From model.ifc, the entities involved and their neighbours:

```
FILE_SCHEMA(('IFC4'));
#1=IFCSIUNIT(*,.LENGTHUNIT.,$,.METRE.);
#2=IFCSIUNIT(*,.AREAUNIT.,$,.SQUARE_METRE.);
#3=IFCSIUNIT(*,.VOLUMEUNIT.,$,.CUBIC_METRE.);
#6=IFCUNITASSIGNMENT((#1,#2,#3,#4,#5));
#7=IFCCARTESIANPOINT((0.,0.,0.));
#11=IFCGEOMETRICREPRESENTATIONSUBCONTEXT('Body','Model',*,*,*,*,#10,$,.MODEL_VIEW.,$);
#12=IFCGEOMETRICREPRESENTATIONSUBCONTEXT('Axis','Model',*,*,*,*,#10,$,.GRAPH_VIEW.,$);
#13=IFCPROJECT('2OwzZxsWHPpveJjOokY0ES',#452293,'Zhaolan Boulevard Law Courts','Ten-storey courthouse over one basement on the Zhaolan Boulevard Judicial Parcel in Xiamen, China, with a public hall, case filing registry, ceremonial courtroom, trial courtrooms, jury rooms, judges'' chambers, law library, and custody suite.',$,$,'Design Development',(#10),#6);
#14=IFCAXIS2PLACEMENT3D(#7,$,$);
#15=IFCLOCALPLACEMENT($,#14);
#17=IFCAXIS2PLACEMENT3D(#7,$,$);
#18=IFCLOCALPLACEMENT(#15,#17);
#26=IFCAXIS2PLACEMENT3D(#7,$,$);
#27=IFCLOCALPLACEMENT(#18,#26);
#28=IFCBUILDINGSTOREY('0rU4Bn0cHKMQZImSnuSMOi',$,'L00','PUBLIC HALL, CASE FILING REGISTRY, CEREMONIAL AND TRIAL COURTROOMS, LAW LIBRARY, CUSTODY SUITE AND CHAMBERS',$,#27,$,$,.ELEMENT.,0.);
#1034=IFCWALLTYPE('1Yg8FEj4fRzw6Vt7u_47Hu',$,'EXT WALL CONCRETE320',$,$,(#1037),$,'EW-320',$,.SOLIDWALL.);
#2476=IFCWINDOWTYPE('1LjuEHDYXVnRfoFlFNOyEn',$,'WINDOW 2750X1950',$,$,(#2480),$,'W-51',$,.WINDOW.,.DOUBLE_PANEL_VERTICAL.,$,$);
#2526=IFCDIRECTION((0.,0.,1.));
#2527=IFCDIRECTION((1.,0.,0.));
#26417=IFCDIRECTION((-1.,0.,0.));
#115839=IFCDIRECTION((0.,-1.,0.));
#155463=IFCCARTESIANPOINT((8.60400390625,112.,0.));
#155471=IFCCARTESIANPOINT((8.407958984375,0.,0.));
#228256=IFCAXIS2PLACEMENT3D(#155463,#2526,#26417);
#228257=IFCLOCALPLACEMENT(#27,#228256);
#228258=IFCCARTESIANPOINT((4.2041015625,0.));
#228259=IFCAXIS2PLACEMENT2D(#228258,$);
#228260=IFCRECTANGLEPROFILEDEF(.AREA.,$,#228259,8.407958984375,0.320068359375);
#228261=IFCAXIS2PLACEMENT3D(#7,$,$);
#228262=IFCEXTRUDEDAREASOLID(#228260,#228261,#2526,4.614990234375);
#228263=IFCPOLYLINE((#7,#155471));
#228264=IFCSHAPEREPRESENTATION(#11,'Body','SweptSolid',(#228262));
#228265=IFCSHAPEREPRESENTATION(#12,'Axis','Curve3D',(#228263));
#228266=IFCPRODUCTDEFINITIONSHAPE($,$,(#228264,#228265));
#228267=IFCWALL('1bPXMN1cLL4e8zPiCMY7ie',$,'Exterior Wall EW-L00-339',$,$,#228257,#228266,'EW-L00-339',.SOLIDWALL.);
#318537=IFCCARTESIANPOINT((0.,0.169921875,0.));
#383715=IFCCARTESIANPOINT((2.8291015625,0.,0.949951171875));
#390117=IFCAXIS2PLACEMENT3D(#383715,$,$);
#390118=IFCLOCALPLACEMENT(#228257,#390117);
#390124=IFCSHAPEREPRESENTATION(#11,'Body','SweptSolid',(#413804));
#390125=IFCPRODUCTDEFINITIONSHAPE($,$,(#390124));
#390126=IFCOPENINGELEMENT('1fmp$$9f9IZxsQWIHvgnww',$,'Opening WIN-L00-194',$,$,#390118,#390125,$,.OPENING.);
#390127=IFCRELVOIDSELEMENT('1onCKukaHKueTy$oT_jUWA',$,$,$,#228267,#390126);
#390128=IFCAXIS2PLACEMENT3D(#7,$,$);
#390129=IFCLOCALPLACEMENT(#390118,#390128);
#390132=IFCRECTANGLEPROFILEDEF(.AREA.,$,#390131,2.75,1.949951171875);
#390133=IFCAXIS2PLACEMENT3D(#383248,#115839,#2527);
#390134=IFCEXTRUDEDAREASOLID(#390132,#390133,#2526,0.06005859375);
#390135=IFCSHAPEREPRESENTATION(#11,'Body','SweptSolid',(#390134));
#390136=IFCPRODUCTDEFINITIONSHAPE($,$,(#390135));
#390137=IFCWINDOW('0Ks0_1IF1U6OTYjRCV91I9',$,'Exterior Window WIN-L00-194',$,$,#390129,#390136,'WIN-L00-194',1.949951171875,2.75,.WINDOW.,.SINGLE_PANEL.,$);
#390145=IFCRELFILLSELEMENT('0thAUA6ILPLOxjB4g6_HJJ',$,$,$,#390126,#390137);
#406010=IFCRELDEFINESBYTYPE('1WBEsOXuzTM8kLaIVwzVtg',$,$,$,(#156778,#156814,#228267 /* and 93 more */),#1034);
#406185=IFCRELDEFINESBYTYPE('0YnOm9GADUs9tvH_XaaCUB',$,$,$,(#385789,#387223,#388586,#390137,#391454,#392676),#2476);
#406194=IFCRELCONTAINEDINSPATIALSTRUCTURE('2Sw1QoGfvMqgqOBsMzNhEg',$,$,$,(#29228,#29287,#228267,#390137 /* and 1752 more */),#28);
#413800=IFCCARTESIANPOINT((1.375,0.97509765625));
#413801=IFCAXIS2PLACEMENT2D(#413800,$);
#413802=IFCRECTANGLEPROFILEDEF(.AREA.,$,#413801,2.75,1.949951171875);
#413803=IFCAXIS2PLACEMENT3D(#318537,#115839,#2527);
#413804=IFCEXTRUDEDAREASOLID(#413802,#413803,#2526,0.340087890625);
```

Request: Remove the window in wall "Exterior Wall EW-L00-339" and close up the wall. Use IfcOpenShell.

```python
import ifcopenshell
import ifcopenshell.api.feature
import ifcopenshell.api.root
import ifcopenshell.geom
import ifcopenshell.util.shape

model = ifcopenshell.open("model.ifc")
settings = ifcopenshell.geom.settings()


def volume(element):
    """Net volume in cubic metres, openings subtracted."""
    shape = ifcopenshell.geom.create_shape(settings, element)
    return ifcopenshell.util.shape.get_volume(shape.geometry)


window = model.by_guid("0Ks0_1IF1U6OTYjRCV91I9")
opening = window.FillsVoids[0].RelatingOpeningElement
wall = opening.VoidsElements[0].RelatingBuildingElement
before = volume(wall)

ifcopenshell.api.root.remove_product(model, product=window)
ifcopenshell.api.feature.remove_feature(model, feature=opening)

after = volume(wall)

print(f"wall volume {before:.3f} -> {after:.3f} m3")

model.write("model_edited.ifc")
```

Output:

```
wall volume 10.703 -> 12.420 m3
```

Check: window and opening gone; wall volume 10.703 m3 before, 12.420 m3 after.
